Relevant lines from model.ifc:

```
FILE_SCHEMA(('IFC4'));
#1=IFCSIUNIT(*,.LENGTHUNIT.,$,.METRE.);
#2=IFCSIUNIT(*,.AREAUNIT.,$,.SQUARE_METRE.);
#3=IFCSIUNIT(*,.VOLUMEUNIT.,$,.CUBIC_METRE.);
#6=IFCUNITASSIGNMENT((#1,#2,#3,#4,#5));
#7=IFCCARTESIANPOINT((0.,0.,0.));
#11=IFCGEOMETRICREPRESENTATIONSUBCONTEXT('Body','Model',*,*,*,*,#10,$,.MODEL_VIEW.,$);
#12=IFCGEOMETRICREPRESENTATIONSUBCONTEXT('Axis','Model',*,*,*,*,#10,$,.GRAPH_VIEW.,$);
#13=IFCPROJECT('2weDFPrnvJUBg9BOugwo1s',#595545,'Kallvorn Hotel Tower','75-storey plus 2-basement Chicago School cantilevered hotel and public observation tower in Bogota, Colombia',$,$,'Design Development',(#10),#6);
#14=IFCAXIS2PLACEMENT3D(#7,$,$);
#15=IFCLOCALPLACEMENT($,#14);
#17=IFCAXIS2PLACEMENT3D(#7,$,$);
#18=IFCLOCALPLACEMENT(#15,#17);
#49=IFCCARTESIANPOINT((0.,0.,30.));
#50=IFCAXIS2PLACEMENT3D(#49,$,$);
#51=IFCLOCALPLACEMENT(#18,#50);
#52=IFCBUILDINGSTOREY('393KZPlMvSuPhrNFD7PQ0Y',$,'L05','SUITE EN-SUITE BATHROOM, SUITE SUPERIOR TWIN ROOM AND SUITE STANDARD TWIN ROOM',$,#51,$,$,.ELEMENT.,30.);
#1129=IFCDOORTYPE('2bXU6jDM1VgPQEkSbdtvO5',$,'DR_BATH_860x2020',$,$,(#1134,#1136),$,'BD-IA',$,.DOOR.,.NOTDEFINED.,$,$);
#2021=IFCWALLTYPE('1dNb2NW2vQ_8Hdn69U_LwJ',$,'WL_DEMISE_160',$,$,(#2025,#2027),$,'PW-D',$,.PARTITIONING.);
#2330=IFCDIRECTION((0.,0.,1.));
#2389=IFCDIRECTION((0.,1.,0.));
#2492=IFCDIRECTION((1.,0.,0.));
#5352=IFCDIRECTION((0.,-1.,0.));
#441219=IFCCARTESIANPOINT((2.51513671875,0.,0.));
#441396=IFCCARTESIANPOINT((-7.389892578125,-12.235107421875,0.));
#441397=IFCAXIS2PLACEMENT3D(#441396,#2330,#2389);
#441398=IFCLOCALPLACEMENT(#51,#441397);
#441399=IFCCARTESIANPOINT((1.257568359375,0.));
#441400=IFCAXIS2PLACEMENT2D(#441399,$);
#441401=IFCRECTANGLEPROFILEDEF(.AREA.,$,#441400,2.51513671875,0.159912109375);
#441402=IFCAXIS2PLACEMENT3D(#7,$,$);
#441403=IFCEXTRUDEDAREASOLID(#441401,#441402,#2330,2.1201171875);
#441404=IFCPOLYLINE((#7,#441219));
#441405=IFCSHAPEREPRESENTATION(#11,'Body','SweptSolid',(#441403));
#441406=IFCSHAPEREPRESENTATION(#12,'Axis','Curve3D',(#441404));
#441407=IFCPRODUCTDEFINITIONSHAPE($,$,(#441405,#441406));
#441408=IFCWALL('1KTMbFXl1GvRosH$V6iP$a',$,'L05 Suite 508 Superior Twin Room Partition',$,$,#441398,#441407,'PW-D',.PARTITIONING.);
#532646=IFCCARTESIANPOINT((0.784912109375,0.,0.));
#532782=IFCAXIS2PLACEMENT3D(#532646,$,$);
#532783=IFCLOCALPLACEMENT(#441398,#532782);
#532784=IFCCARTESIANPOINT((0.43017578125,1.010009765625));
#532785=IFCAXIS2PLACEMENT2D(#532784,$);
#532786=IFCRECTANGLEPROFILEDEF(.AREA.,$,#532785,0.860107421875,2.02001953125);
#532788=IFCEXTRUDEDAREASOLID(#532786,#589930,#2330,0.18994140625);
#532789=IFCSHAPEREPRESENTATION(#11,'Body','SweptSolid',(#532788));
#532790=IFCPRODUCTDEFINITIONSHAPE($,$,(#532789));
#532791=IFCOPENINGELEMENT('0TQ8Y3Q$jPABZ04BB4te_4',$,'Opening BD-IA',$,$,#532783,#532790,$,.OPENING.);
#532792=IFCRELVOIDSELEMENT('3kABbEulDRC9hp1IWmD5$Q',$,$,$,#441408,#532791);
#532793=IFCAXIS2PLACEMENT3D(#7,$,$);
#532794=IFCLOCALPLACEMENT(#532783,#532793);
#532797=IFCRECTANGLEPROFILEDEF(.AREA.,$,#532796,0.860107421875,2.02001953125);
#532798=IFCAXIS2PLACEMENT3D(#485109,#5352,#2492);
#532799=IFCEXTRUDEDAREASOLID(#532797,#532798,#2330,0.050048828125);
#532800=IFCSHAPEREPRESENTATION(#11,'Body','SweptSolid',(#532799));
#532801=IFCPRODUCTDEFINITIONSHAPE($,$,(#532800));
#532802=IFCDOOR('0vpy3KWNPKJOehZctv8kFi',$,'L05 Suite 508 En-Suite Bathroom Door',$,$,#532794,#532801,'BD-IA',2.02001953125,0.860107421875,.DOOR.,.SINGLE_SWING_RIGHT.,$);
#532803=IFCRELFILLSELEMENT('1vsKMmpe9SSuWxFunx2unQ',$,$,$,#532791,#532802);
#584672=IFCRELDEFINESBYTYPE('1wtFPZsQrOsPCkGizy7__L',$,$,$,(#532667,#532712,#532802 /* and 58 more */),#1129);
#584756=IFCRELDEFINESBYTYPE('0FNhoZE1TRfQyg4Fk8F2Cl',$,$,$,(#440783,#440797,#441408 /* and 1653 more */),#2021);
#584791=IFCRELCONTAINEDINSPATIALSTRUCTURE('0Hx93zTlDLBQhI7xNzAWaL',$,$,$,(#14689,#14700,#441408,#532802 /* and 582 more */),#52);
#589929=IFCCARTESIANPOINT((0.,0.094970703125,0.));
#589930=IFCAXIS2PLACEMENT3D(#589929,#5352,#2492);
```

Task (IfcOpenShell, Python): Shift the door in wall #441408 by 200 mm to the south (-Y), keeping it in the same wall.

```python
import ifcopenshell
import ifcopenshell.api.geometry
import ifcopenshell.util.placement

model = ifcopenshell.open("model.ifc")

door = model.by_guid("0vpy3KWNPKJOehZctv8kFi")
opening = door.FillsVoids[0].RelatingOpeningElement
wall = opening.VoidsElements[0].RelatingBuildingElement

wall_matrix = ifcopenshell.util.placement.get_local_placement(wall.ObjectPlacement)
shift = wall_matrix[:3, 0] * -0.2
before = ifcopenshell.util.placement.get_local_placement(door.ObjectPlacement)[:3, 3].copy()

# The door is placed relative to its opening, so it follows when the opening moves.
matrix = ifcopenshell.util.placement.get_local_placement(opening.ObjectPlacement)
matrix[:3, 3] += shift
ifcopenshell.api.geometry.edit_object_placement(
    model, product=opening, matrix=matrix, is_si=False, should_transform_children=True
)

after = ifcopenshell.util.placement.get_local_placement(door.ObjectPlacement)[:3, 3]
print("door moved by", (after - before).round(3) + 0.0)

model.write("model_rev.ifc")
```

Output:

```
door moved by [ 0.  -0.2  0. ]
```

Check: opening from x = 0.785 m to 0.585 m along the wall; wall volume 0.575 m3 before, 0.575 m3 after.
